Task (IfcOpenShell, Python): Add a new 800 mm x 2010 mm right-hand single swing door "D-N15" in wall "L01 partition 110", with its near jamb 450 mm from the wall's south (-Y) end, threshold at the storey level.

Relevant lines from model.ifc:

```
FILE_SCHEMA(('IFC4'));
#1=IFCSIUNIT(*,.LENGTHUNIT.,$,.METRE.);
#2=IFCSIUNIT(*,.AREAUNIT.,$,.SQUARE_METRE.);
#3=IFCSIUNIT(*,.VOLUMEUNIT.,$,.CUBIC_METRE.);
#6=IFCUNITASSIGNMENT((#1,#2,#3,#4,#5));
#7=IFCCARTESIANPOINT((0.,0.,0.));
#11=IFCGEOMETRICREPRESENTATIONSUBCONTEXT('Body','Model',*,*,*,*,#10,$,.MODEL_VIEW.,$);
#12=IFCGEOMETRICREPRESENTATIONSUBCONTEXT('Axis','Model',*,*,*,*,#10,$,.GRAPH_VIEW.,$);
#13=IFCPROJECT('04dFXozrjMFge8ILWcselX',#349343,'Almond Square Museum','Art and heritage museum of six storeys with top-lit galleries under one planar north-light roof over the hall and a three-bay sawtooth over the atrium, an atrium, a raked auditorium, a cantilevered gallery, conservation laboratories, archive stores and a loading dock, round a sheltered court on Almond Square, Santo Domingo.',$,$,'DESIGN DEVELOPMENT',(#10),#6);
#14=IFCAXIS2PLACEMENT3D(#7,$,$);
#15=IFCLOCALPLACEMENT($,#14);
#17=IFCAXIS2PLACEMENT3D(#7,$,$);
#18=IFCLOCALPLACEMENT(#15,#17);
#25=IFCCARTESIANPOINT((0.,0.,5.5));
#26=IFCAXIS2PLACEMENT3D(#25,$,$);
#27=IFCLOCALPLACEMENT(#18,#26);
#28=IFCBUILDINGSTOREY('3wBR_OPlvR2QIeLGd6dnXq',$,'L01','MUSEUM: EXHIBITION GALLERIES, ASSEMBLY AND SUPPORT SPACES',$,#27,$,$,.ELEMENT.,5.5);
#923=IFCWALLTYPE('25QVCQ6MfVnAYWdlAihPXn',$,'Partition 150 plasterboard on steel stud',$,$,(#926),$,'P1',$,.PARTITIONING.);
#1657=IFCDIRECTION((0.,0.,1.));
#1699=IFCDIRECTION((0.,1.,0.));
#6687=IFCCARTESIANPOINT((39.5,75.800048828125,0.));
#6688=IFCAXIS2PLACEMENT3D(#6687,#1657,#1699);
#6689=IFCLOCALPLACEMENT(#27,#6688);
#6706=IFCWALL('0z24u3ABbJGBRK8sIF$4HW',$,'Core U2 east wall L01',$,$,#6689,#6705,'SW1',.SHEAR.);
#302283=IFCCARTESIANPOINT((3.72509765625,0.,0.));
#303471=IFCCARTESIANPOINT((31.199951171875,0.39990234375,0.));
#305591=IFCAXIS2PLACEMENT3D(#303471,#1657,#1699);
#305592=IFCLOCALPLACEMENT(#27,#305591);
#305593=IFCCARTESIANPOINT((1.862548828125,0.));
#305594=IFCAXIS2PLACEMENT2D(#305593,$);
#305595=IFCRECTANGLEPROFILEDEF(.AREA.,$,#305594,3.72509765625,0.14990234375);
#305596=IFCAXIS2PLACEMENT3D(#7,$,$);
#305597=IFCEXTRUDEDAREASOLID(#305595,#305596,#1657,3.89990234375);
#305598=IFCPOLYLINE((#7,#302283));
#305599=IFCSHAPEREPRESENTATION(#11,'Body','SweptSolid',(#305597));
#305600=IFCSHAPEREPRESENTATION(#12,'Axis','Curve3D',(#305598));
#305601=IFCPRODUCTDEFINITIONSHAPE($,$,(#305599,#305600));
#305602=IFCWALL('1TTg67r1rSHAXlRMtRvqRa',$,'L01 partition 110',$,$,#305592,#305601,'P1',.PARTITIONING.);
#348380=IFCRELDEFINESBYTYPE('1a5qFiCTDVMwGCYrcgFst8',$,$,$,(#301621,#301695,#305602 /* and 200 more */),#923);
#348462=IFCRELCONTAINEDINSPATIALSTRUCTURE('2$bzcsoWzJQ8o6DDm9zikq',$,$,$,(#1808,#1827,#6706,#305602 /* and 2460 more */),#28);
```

```python
import numpy as np
import ifcopenshell
import ifcopenshell.api.feature
import ifcopenshell.api.geometry
import ifcopenshell.api.root
import ifcopenshell.api.spatial
import ifcopenshell.geom
import ifcopenshell.util.element
import ifcopenshell.util.placement
import ifcopenshell.util.representation
import ifcopenshell.util.shape
import ifcopenshell.util.unit

model = ifcopenshell.open("model.ifc")
unit_scale = ifcopenshell.util.unit.calculate_unit_scale(model)
settings = ifcopenshell.geom.settings()


def volume(element):
    """Net volume in cubic metres, openings subtracted."""
    shape = ifcopenshell.geom.create_shape(settings, element)
    return ifcopenshell.util.shape.get_volume(shape.geometry)


wall = model.by_guid("1TTg67r1rSHAXlRMtRvqRa")
storey = ifcopenshell.util.element.get_container(wall, ifc_class="IfcBuildingStorey")
context = ifcopenshell.util.representation.get_context(model, "Model", "Body", "MODEL_VIEW")
before = volume(wall)

width, height, from_end, sill = 0.8, 2.01, 0.45, 0.0  # metres

# The wall runs along its own X axis, and the end named is its -X end.
wall_shape = ifcopenshell.geom.create_shape(settings, wall)
x, y, z = ifcopenshell.util.shape.get_vertices(wall_shape.geometry).T
start = x.min() + from_end
face, thickness = float(y.min()), float(y.max() - y.min())
wall_matrix = ifcopenshell.util.placement.get_local_placement(wall.ObjectPlacement)
level = ifcopenshell.util.placement.get_local_placement(storey.ObjectPlacement)[2, 3]


def in_wall(x, y):
    """Placement at x, y metres in the wall's axes, at sill height."""
    matrix = wall_matrix.copy()
    matrix[:, 3] = wall_matrix @ np.array([x / unit_scale, y / unit_scale, 0.0, 1.0])
    matrix[2, 3] = level + sill / unit_scale
    return matrix


# Opening: a box that overshoots both wall faces by 50 mm.
opening = ifcopenshell.api.root.create_entity(model, ifc_class="IfcOpeningElement", predefined_type="OPENING")
box = ifcopenshell.api.geometry.add_wall_representation(
    model, context=context, length=width, height=height, thickness=thickness + 0.1
)
ifcopenshell.api.geometry.assign_representation(model, product=opening, representation=box)
ifcopenshell.api.geometry.edit_object_placement(model, product=opening, matrix=in_wall(start, face - 0.05), is_si=False)
ifcopenshell.api.feature.add_feature(model, feature=opening, element=wall)

door = ifcopenshell.api.root.create_entity(model, ifc_class="IfcDoor", name="D-N15", predefined_type="DOOR")
door.OverallWidth, door.OverallHeight = width / unit_scale, height / unit_scale
door.OperationType = "SINGLE_SWING_RIGHT"
body = ifcopenshell.api.geometry.add_door_representation(
    model,
    context=context,
    overall_width=door.OverallWidth,
    overall_height=door.OverallHeight,
    operation_type="SINGLE_SWING_RIGHT",
    lining_properties={"LiningDepth": thickness / unit_scale, "ThresholdDepth": thickness / unit_scale},
)
ifcopenshell.api.geometry.assign_representation(model, product=door, representation=body)
ifcopenshell.api.spatial.assign_container(model, products=[door], relating_structure=storey)
ifcopenshell.api.feature.add_filling(model, opening=opening, element=door)

# The lining spans the wall, so the door starts at the wall face.
ifcopenshell.api.geometry.edit_object_placement(model, product=door, matrix=in_wall(start, face), is_si=False)

after = volume(wall)

print(f"wall volume {before:.3f} -> {after:.3f} m3")

model.write("model_edited.ifc")
```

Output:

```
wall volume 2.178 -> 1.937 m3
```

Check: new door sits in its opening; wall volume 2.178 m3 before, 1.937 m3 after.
